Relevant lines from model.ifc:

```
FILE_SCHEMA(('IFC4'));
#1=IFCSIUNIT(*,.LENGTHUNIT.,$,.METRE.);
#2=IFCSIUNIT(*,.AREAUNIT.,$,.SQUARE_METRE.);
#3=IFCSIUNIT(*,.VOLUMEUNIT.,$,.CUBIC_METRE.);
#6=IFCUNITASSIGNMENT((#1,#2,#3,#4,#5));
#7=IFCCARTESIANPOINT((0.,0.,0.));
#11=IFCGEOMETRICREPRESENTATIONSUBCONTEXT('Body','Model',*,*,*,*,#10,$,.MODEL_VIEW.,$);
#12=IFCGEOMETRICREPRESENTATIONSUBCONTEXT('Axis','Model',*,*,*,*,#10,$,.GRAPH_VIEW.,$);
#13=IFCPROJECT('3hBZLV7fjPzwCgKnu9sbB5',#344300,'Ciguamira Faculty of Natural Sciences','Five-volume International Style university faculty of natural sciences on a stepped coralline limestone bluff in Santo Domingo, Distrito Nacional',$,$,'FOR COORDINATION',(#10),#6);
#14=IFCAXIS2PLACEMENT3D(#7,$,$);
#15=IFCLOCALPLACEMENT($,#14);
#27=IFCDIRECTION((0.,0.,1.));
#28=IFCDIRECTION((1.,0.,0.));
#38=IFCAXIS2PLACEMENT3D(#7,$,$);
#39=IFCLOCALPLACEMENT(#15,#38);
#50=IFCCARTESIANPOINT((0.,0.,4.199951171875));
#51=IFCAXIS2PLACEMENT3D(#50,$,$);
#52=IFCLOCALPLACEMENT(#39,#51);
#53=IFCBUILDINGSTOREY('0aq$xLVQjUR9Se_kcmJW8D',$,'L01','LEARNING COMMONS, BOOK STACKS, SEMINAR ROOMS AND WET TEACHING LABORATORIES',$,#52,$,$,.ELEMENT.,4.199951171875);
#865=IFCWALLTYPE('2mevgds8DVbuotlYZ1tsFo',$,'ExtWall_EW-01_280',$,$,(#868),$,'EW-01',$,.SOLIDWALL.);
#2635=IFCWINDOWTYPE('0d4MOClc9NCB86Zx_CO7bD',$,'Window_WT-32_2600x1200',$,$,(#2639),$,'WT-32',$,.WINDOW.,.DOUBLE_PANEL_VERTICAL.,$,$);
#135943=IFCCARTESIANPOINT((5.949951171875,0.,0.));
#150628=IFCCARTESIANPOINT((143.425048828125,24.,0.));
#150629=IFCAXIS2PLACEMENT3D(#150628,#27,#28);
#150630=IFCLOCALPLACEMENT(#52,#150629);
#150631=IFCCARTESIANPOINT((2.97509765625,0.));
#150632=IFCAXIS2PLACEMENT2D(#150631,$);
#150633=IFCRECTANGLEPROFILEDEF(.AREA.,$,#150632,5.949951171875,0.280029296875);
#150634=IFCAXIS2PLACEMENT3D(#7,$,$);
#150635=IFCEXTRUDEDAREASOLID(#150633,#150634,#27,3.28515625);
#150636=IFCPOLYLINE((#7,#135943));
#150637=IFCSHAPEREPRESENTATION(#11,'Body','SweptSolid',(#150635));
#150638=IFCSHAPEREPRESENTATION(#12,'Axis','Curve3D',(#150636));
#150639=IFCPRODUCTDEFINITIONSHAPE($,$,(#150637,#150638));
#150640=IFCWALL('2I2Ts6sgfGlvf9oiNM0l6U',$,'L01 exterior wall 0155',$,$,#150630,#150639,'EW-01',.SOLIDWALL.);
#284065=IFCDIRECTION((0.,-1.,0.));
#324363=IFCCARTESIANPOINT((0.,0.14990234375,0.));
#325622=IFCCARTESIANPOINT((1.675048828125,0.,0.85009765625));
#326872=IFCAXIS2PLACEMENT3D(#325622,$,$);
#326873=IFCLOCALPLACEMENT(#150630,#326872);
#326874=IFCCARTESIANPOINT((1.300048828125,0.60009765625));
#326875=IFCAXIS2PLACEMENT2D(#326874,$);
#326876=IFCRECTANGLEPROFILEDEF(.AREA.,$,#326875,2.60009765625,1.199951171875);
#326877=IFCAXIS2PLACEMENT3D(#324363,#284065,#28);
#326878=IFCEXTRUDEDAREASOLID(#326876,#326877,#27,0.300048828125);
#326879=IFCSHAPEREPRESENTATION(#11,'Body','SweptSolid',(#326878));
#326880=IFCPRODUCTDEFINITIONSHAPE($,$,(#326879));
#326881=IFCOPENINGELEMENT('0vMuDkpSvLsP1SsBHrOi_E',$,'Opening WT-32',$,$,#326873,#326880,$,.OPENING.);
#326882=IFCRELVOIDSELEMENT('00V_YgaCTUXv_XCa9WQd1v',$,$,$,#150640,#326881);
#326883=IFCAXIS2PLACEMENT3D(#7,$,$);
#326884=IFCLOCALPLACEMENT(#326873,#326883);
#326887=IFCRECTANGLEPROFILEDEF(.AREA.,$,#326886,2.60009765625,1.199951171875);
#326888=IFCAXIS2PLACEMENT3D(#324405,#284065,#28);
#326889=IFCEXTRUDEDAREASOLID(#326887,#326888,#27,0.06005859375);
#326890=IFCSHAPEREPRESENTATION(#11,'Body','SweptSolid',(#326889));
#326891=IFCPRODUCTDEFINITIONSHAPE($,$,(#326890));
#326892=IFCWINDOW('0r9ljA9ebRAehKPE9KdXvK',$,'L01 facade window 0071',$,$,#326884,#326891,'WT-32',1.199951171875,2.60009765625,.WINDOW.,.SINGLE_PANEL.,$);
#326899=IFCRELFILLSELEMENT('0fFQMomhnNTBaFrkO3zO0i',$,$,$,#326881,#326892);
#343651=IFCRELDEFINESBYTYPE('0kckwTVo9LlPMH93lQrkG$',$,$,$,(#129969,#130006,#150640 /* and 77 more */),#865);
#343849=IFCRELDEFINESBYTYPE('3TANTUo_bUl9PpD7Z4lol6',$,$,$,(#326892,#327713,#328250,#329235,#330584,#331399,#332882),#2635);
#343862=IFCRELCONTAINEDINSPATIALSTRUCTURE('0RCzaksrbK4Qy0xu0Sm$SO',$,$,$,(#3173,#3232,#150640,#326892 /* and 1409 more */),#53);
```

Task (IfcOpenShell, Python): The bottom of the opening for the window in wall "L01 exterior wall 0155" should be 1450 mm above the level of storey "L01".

```python
import numpy as np
import ifcopenshell
import ifcopenshell.api.geometry
import ifcopenshell.geom
import ifcopenshell.util.element
import ifcopenshell.util.placement
import ifcopenshell.util.shape
import ifcopenshell.util.unit

model = ifcopenshell.open("model.ifc")
unit_scale = ifcopenshell.util.unit.calculate_unit_scale(model)

window = model.by_guid("0r9ljA9ebRAehKPE9KdXvK")
opening = window.FillsVoids[0].RelatingOpeningElement
storey = ifcopenshell.util.element.get_container(window, ifc_class="IfcBuildingStorey")
level = ifcopenshell.util.placement.get_local_placement(storey.ObjectPlacement)[2, 3]

# The opening's origin need not be at the sill, so measure its lowest point.
shape = ifcopenshell.geom.create_shape(ifcopenshell.geom.settings(), opening)
bottom = ifcopenshell.util.shape.get_shape_bottom_elevation(shape, shape.geometry) / unit_scale
dz = level + 1.45 - bottom

shift = np.array([0.0, 0.0, dz])
# The window is placed relative to its opening, so it follows when the opening moves.
matrix = ifcopenshell.util.placement.get_local_placement(opening.ObjectPlacement)
matrix[:3, 3] += shift
ifcopenshell.api.geometry.edit_object_placement(
    model, product=opening, matrix=matrix, is_si=False, should_transform_children=True
)

print(f"moved by {dz * unit_scale:+.3f} m")

model.write("model_v2.ifc")
```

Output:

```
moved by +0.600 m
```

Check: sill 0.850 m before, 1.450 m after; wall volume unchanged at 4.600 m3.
